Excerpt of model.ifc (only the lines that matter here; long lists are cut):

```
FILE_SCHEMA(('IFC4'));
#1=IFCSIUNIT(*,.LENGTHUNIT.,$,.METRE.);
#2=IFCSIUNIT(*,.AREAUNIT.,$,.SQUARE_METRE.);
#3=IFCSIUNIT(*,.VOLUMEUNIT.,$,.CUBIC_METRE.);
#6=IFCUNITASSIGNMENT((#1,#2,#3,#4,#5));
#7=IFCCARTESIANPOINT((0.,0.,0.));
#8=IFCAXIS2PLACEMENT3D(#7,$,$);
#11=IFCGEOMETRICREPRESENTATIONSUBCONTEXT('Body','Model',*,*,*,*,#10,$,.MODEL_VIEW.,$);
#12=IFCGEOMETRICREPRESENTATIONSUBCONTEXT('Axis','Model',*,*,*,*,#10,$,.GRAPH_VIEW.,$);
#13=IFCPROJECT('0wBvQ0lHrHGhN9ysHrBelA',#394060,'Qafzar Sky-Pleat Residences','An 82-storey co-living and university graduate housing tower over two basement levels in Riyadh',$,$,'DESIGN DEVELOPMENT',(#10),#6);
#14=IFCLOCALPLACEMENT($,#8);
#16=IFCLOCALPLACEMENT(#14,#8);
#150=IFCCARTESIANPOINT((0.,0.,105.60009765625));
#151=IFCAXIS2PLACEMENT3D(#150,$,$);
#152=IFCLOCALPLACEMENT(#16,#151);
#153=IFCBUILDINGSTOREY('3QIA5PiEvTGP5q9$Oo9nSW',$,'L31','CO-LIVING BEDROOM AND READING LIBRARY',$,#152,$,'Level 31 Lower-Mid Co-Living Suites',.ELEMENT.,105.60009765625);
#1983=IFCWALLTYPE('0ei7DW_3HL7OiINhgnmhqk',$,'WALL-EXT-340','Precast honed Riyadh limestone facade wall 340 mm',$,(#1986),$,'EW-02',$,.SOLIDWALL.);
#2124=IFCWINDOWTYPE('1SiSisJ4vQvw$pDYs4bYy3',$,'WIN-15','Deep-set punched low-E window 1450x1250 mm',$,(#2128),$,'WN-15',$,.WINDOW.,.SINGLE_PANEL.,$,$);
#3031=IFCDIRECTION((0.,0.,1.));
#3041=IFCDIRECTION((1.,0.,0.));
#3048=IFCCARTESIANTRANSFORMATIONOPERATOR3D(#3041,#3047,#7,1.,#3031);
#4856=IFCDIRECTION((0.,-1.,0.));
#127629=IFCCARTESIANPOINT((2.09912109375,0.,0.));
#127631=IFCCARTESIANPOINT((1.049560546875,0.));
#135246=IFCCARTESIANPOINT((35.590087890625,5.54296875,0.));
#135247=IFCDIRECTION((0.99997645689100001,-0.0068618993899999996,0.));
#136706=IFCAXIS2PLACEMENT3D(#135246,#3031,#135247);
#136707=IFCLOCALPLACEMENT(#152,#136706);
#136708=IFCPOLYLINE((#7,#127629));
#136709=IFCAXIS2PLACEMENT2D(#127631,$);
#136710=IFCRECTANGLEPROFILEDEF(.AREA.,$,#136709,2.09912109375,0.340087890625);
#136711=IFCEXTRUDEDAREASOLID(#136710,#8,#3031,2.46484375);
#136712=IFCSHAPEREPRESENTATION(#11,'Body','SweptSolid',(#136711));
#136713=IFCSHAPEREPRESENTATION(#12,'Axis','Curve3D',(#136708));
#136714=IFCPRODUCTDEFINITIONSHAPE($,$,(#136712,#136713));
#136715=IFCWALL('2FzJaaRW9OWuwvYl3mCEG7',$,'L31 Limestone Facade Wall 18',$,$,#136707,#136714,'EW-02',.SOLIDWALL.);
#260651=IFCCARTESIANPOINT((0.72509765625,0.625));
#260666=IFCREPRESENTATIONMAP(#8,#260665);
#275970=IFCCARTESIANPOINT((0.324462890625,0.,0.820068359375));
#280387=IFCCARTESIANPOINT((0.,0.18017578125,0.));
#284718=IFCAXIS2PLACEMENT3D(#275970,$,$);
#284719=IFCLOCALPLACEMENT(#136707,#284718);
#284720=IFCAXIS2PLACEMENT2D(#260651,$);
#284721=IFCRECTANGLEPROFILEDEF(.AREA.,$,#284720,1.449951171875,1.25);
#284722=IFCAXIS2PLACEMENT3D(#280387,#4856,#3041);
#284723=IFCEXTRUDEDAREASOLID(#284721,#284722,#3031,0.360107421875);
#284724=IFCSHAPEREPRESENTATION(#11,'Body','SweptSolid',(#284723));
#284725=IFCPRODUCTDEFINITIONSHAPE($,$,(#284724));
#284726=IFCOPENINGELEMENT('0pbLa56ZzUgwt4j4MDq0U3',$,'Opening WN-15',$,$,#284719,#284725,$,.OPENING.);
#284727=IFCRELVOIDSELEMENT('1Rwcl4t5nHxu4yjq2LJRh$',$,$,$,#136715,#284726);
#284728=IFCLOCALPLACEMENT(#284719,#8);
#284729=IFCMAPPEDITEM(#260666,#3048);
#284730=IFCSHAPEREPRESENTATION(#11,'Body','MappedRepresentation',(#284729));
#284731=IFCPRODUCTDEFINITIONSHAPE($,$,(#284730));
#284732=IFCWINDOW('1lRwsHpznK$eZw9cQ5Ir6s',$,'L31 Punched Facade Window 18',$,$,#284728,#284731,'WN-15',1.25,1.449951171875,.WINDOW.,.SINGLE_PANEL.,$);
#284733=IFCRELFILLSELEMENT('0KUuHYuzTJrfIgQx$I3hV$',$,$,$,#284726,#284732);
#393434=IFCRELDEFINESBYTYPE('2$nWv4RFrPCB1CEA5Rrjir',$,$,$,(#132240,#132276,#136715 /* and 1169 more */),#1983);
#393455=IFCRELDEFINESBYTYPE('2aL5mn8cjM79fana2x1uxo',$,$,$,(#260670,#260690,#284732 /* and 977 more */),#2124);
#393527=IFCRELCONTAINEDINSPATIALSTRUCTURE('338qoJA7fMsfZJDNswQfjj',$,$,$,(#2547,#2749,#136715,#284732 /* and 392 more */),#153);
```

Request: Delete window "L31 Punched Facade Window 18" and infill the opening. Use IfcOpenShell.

```python
import ifcopenshell
import ifcopenshell.api.feature
import ifcopenshell.api.root
import ifcopenshell.geom
import ifcopenshell.util.shape

model = ifcopenshell.open("model.ifc")
settings = ifcopenshell.geom.settings()


def volume(element):
    """Net volume in cubic metres, openings subtracted."""
    shape = ifcopenshell.geom.create_shape(settings, element)
    return ifcopenshell.util.shape.get_volume(shape.geometry)


window = model.by_id(284732)
opening = window.FillsVoids[0].RelatingOpeningElement
wall = opening.VoidsElements[0].RelatingBuildingElement
before = volume(wall)

ifcopenshell.api.root.remove_product(model, product=window)
ifcopenshell.api.feature.remove_feature(model, feature=opening)

after = volume(wall)

print(f"wall volume {before:.3f} -> {after:.3f} m3")

model.write("model_updated.ifc")
```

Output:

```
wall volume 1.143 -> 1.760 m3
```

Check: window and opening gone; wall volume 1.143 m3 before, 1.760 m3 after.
